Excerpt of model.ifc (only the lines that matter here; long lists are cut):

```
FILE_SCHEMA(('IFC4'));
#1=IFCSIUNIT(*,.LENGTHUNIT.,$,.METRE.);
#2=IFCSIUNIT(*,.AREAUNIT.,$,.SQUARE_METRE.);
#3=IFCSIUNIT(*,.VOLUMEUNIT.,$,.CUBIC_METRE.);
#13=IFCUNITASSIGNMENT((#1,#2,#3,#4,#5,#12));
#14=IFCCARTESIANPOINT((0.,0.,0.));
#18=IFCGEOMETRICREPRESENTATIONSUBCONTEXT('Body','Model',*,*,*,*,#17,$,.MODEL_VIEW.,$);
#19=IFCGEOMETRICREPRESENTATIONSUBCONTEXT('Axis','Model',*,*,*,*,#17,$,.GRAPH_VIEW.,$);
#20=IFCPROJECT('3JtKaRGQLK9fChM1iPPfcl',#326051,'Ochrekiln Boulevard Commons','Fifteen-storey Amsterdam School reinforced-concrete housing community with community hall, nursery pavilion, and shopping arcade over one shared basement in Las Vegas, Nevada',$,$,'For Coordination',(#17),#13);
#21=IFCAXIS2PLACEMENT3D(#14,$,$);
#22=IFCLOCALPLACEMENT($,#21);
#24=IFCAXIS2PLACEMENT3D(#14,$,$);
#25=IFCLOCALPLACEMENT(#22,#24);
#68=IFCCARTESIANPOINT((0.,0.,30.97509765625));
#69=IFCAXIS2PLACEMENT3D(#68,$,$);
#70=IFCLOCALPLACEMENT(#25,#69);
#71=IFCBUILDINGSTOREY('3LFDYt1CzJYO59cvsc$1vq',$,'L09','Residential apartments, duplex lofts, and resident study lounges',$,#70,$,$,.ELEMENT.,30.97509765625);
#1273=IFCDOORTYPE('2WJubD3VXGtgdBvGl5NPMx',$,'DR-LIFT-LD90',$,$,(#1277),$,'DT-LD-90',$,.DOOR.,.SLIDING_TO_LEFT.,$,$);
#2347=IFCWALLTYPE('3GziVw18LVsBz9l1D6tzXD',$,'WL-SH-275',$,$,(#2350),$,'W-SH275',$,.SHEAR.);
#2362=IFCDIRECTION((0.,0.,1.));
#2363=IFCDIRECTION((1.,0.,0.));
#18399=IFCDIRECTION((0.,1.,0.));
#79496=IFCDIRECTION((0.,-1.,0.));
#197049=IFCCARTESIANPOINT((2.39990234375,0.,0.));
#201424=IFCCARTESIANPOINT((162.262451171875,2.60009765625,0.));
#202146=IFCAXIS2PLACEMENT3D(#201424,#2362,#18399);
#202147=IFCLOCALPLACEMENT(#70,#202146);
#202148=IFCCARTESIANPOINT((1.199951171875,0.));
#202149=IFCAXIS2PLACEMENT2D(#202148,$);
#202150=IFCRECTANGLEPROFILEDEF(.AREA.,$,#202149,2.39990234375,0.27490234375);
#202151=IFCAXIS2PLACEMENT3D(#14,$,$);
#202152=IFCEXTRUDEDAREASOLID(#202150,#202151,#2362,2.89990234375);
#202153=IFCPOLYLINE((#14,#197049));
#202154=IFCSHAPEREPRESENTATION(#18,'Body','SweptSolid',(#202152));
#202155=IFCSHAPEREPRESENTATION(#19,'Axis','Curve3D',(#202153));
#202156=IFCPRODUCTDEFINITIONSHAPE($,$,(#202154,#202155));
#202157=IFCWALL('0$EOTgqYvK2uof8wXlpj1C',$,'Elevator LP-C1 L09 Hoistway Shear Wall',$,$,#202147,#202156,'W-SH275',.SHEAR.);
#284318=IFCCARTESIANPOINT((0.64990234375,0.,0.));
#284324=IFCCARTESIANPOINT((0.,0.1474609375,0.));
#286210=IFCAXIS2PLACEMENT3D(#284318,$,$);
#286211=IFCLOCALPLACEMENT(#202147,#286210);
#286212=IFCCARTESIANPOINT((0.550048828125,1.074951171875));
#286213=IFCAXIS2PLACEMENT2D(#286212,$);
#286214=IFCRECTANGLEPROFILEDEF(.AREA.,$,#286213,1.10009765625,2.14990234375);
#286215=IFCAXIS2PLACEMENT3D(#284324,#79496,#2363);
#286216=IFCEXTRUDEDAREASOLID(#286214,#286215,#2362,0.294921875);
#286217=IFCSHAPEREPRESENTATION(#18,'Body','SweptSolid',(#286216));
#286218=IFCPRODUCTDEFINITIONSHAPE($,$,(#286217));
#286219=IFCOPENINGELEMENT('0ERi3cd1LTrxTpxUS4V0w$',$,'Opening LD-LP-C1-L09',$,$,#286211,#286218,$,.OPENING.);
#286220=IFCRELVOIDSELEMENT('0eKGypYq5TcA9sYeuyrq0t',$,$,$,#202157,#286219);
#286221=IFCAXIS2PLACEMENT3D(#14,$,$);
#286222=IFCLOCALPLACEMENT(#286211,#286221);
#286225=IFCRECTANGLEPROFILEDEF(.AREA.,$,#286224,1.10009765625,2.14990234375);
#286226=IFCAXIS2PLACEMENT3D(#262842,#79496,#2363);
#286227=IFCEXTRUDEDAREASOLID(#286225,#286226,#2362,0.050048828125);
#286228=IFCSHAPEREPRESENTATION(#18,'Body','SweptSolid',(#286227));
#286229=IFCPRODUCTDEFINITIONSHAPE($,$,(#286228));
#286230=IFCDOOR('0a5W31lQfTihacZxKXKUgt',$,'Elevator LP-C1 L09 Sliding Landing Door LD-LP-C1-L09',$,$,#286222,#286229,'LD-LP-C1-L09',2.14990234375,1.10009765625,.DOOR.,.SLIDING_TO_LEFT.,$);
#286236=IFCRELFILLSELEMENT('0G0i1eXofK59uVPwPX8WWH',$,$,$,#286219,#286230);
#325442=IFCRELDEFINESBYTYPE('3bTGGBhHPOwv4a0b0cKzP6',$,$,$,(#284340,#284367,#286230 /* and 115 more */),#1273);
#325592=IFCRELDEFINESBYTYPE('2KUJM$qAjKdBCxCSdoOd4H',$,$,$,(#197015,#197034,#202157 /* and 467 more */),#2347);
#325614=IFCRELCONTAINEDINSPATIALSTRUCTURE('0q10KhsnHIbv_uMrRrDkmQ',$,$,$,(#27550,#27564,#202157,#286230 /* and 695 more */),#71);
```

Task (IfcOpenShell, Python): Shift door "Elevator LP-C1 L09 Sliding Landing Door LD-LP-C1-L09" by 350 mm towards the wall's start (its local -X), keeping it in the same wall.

```python
import ifcopenshell
import ifcopenshell.api.geometry
import ifcopenshell.util.placement

model = ifcopenshell.open("model.ifc")

door = model.by_guid("0a5W31lQfTihacZxKXKUgt")
opening = door.FillsVoids[0].RelatingOpeningElement
wall = opening.VoidsElements[0].RelatingBuildingElement

wall_matrix = ifcopenshell.util.placement.get_local_placement(wall.ObjectPlacement)
shift = wall_matrix[:3, 0] * -0.35
before = ifcopenshell.util.placement.get_local_placement(door.ObjectPlacement)[:3, 3].copy()

# The door is placed relative to its opening, so it follows when the opening moves.
matrix = ifcopenshell.util.placement.get_local_placement(opening.ObjectPlacement)
matrix[:3, 3] += shift
ifcopenshell.api.geometry.edit_object_placement(
    model, product=opening, matrix=matrix, is_si=False, should_transform_children=True
)

after = ifcopenshell.util.placement.get_local_placement(door.ObjectPlacement)[:3, 3]
print("door moved by", (after - before).round(3) + 0.0)

model.write("model_updated.ifc")
```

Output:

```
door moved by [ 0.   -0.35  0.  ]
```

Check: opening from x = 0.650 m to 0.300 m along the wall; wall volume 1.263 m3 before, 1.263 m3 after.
